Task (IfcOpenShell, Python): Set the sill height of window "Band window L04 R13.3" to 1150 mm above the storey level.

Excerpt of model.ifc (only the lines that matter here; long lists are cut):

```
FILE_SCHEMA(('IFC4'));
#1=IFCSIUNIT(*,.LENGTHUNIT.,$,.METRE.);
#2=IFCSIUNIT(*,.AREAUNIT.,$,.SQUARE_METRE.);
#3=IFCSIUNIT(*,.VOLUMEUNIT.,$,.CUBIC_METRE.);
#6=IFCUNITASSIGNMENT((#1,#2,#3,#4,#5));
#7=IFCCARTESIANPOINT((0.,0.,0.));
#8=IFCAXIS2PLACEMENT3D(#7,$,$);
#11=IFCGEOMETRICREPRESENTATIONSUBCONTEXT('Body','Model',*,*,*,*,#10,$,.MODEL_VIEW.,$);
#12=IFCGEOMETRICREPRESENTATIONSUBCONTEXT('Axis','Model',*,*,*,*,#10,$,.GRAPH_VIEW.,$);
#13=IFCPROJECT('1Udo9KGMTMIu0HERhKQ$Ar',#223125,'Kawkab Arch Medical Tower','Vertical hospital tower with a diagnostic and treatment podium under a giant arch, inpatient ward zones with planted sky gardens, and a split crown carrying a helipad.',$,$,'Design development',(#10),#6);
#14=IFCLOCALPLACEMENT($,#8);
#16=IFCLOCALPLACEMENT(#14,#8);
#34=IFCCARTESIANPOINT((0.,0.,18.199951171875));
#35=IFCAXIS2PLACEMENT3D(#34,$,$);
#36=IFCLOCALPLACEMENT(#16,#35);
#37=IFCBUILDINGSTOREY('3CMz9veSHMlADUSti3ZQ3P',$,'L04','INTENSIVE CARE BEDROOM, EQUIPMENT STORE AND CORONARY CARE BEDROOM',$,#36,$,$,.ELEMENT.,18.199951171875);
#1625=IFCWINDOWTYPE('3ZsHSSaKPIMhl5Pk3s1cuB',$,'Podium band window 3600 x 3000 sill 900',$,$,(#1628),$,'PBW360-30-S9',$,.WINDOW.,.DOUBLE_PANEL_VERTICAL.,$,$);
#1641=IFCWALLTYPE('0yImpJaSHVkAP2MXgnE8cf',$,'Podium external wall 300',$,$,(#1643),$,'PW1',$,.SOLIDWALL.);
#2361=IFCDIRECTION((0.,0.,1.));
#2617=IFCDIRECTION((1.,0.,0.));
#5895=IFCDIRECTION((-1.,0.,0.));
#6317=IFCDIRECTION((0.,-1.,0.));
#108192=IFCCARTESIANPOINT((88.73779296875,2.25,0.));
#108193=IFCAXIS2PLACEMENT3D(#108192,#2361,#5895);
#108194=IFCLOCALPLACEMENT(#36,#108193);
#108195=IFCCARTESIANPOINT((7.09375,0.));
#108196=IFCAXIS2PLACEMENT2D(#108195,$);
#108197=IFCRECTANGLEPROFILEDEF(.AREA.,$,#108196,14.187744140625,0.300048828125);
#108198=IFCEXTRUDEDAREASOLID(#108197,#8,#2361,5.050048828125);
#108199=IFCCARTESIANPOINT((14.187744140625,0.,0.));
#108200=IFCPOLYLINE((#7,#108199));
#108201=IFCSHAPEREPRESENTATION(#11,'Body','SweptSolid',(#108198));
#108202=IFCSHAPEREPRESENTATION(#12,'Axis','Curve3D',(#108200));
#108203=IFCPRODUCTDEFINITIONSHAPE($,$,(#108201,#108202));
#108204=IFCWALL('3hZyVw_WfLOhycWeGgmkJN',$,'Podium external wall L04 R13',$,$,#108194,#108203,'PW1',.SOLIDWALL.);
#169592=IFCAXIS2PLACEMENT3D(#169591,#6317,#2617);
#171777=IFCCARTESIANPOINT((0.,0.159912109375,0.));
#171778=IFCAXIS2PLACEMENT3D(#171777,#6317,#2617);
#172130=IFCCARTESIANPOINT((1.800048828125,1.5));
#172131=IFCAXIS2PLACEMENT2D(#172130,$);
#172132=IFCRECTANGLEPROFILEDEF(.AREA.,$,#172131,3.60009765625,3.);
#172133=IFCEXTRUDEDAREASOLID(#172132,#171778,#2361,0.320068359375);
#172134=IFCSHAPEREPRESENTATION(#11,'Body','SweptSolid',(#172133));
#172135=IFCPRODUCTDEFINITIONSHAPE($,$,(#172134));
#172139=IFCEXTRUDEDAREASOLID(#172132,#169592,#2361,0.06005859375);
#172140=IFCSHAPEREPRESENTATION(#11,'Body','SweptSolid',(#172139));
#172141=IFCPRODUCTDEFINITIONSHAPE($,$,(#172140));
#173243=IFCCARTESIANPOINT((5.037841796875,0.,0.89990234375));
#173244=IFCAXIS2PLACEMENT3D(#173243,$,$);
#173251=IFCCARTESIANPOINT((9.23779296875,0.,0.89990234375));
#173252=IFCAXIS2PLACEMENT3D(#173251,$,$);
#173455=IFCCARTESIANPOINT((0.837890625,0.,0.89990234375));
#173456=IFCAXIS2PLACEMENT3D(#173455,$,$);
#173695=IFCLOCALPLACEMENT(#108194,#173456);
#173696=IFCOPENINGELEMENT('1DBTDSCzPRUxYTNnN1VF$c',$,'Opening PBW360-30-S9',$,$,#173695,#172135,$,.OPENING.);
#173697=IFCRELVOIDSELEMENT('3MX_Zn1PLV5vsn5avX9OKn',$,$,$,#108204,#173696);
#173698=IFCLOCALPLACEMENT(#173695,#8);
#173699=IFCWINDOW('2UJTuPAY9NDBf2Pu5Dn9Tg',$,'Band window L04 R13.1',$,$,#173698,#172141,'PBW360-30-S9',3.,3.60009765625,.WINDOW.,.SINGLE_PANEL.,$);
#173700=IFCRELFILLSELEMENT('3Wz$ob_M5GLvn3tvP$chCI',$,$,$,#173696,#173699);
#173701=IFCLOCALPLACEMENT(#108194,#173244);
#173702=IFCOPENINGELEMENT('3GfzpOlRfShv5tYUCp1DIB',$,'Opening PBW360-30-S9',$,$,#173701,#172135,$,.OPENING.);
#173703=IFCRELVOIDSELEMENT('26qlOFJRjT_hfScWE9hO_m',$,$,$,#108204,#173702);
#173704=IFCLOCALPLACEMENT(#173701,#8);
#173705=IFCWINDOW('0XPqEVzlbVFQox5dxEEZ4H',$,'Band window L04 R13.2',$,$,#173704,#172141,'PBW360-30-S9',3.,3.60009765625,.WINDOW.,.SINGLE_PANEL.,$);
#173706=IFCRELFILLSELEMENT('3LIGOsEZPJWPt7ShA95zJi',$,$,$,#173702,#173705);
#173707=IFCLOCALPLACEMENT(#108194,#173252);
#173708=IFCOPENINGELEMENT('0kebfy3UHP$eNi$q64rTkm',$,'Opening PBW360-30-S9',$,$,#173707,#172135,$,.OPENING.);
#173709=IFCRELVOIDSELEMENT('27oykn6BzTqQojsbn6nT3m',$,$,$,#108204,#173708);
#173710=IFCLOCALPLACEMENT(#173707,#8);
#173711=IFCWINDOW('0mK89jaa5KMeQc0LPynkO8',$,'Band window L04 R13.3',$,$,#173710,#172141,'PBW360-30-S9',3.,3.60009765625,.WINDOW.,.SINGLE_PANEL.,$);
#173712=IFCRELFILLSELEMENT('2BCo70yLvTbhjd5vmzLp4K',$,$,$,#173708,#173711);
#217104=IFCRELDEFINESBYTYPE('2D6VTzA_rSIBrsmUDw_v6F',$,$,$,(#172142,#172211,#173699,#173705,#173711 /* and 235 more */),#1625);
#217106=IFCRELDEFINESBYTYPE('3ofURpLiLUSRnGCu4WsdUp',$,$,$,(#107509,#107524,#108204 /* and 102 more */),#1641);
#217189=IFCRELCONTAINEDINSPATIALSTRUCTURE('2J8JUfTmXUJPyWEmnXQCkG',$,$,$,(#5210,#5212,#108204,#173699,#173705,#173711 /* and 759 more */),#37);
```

```python
import numpy as np
import ifcopenshell
import ifcopenshell.api.geometry
import ifcopenshell.geom
import ifcopenshell.util.element
import ifcopenshell.util.placement
import ifcopenshell.util.shape
import ifcopenshell.util.unit

model = ifcopenshell.open("model.ifc")
unit_scale = ifcopenshell.util.unit.calculate_unit_scale(model)

window = model.by_guid("0mK89jaa5KMeQc0LPynkO8")
opening = window.FillsVoids[0].RelatingOpeningElement
storey = ifcopenshell.util.element.get_container(window, ifc_class="IfcBuildingStorey")
level = ifcopenshell.util.placement.get_local_placement(storey.ObjectPlacement)[2, 3]

# The opening's origin need not be at the sill, so measure its lowest point.
shape = ifcopenshell.geom.create_shape(ifcopenshell.geom.settings(), opening)
bottom = ifcopenshell.util.shape.get_shape_bottom_elevation(shape, shape.geometry) / unit_scale
dz = level + 1.15 / unit_scale - bottom

shift = np.array([0.0, 0.0, dz])
# The window is placed relative to its opening, so it follows when the opening moves.
matrix = ifcopenshell.util.placement.get_local_placement(opening.ObjectPlacement)
matrix[:3, 3] += shift
ifcopenshell.api.geometry.edit_object_placement(
    model, product=opening, matrix=matrix, is_si=False, should_transform_children=True
)

print(f"moved by {dz * unit_scale:+.3f} m")

model.write("model_updated.ifc")
```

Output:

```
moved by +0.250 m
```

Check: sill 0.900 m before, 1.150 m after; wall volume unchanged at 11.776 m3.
